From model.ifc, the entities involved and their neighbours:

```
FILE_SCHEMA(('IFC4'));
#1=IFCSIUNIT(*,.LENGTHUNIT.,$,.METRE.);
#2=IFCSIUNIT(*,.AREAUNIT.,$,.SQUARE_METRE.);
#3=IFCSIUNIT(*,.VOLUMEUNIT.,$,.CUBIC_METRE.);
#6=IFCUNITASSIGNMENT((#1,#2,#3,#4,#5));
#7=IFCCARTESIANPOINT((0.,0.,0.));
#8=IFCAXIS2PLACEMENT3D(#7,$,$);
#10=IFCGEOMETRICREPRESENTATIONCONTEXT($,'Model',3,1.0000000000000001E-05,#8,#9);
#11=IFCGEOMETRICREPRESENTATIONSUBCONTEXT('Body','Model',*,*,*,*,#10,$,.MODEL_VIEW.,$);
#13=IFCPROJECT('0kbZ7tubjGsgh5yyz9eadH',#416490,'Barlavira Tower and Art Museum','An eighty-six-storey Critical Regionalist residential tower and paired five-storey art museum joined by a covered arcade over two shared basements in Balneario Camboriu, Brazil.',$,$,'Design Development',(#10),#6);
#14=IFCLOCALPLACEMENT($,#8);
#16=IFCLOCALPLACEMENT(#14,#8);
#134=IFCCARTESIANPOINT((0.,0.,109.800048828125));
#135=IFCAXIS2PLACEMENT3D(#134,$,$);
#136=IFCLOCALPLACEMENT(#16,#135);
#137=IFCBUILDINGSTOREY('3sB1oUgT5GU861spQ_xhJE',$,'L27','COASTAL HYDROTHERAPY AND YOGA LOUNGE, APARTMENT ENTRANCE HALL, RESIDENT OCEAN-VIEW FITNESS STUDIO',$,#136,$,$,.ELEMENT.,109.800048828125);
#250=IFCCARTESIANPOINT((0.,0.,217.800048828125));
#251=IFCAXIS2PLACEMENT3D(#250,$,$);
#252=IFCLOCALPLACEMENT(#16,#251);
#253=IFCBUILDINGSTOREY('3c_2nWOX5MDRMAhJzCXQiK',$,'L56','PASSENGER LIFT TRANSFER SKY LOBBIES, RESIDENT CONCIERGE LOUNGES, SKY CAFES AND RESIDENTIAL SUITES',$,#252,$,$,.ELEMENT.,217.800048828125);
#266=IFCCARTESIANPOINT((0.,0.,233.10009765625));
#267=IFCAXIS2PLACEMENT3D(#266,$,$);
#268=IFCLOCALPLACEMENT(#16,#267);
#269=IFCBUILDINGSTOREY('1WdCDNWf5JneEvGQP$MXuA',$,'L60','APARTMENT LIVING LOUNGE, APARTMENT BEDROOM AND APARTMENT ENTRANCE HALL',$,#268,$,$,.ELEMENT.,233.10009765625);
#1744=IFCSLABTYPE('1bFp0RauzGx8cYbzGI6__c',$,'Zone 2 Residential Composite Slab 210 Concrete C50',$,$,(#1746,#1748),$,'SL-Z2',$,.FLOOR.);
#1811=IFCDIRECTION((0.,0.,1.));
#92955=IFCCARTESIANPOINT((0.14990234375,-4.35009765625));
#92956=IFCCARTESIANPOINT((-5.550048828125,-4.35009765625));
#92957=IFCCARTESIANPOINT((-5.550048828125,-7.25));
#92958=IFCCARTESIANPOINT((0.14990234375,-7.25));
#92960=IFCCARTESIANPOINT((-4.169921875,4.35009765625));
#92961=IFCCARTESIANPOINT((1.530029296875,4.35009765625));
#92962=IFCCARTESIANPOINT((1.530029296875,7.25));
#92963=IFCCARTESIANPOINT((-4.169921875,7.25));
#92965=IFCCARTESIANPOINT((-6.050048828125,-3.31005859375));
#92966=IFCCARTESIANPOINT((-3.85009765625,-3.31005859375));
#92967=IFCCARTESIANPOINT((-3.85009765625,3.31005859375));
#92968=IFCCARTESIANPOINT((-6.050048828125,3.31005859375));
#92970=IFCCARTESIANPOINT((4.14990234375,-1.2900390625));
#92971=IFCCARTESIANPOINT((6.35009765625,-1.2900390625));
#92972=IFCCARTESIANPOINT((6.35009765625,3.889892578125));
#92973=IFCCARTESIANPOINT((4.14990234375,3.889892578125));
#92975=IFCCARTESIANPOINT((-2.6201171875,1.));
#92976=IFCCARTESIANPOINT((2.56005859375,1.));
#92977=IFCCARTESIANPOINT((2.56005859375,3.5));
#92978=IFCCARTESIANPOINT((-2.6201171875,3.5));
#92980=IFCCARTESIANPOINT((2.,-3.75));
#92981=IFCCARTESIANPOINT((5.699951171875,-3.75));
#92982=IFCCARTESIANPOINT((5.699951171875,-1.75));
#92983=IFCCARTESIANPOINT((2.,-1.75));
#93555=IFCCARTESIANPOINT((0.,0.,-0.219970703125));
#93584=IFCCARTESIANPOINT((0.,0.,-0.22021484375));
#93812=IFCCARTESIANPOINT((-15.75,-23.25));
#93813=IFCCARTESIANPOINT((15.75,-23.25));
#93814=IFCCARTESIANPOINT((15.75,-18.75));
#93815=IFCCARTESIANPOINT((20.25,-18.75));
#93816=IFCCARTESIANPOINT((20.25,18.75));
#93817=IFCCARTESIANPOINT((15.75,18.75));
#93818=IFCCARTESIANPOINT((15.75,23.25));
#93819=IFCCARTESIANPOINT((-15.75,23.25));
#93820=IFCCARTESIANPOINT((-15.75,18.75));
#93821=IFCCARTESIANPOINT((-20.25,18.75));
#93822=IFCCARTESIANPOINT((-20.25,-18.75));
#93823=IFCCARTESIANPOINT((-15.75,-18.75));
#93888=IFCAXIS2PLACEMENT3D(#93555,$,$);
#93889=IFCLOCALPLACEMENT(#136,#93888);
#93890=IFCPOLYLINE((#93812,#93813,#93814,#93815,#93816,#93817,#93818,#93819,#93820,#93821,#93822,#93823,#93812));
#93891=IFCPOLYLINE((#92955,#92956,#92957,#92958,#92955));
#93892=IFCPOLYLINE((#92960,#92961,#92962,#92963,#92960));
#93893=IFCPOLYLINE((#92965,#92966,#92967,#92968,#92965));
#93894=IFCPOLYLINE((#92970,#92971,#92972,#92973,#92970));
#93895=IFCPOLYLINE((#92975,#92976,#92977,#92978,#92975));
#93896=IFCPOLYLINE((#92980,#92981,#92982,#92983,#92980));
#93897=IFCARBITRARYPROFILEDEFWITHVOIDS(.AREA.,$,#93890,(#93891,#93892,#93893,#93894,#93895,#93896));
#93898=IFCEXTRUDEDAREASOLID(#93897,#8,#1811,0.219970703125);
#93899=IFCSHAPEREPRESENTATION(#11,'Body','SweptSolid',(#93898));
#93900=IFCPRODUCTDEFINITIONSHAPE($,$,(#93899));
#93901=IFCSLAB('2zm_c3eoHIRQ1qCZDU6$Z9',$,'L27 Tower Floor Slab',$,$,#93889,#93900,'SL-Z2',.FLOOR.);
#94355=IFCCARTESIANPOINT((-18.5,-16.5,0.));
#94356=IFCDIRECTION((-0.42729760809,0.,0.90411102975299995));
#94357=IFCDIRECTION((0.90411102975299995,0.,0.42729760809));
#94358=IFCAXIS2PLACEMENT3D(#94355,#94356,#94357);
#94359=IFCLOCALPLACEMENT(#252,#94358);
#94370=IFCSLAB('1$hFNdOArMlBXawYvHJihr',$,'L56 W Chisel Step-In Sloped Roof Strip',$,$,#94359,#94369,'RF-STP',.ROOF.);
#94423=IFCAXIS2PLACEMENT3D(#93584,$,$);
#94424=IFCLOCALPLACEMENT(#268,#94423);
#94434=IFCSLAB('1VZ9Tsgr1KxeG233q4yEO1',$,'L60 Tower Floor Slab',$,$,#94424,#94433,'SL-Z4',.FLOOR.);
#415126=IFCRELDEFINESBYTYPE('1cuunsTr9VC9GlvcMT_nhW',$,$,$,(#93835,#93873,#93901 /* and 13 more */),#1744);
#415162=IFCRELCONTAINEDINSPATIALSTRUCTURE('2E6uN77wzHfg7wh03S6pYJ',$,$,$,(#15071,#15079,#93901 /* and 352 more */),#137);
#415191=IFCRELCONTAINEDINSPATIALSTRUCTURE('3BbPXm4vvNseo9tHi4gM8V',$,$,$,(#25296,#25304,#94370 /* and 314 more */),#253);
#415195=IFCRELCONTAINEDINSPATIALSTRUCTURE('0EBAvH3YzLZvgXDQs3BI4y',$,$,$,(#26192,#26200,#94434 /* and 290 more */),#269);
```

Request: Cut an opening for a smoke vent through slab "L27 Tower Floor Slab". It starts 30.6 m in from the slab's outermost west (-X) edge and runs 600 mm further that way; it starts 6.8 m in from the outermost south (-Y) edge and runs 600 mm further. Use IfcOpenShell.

```python
import numpy as np
import ifcopenshell
import ifcopenshell.api.feature
import ifcopenshell.api.geometry
import ifcopenshell.api.root
import ifcopenshell.geom
import ifcopenshell.util.placement
import ifcopenshell.util.representation
import ifcopenshell.util.shape
import ifcopenshell.util.unit

model = ifcopenshell.open("model.ifc")
unit_scale = ifcopenshell.util.unit.calculate_unit_scale(model)
settings = ifcopenshell.geom.settings()


def volume(element):
    """Net volume in cubic metres, openings subtracted."""
    shape = ifcopenshell.geom.create_shape(settings, element)
    return ifcopenshell.util.shape.get_volume(shape.geometry)


slab = model.by_guid("2zm_c3eoHIRQ1qCZDU6$Z9")
before = volume(slab)

# Extent in the slab's own axes, in metres. The edges named are its -X and -Y sides.
slab_shape = ifcopenshell.geom.create_shape(settings, slab)
vertices = ifcopenshell.util.shape.get_vertices(slab_shape.geometry)
x_min, y_min, bottom = vertices.min(axis=0)
top = vertices[:, 2].max()

opening = ifcopenshell.api.root.create_entity(model, ifc_class="IfcOpeningElement", name="Smoke vent opening", predefined_type="OPENING")
context = ifcopenshell.util.representation.get_context(model, "Model", "Body", "MODEL_VIEW")
width, depth = 0.6, 0.6
outline = [(0.0, 0.0), (width, 0.0), (width, depth), (0.0, depth), (0.0, 0.0)]
# Overshoot both faces by 50 mm so the cut is clean.
shape = ifcopenshell.api.geometry.add_slab_representation(
    model, context=context, depth=top - bottom + 0.1, polyline=outline
)
ifcopenshell.api.geometry.assign_representation(model, product=opening, representation=shape)

matrix = ifcopenshell.util.placement.get_local_placement(slab.ObjectPlacement)
matrix[:, 3] = matrix @ np.append(np.array([x_min + 30.6, y_min + 6.8, bottom - 0.05]) / unit_scale, 1.0)
ifcopenshell.api.geometry.edit_object_placement(model, product=opening, matrix=matrix, is_si=False)
ifcopenshell.api.feature.add_feature(model, feature=opening, element=slab)

after = volume(slab)

print(f"slab volume {before:.3f} -> {after:.3f} m3")

model.write("model-out.ifc")
```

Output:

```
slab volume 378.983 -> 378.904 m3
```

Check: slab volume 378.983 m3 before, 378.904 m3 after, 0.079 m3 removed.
